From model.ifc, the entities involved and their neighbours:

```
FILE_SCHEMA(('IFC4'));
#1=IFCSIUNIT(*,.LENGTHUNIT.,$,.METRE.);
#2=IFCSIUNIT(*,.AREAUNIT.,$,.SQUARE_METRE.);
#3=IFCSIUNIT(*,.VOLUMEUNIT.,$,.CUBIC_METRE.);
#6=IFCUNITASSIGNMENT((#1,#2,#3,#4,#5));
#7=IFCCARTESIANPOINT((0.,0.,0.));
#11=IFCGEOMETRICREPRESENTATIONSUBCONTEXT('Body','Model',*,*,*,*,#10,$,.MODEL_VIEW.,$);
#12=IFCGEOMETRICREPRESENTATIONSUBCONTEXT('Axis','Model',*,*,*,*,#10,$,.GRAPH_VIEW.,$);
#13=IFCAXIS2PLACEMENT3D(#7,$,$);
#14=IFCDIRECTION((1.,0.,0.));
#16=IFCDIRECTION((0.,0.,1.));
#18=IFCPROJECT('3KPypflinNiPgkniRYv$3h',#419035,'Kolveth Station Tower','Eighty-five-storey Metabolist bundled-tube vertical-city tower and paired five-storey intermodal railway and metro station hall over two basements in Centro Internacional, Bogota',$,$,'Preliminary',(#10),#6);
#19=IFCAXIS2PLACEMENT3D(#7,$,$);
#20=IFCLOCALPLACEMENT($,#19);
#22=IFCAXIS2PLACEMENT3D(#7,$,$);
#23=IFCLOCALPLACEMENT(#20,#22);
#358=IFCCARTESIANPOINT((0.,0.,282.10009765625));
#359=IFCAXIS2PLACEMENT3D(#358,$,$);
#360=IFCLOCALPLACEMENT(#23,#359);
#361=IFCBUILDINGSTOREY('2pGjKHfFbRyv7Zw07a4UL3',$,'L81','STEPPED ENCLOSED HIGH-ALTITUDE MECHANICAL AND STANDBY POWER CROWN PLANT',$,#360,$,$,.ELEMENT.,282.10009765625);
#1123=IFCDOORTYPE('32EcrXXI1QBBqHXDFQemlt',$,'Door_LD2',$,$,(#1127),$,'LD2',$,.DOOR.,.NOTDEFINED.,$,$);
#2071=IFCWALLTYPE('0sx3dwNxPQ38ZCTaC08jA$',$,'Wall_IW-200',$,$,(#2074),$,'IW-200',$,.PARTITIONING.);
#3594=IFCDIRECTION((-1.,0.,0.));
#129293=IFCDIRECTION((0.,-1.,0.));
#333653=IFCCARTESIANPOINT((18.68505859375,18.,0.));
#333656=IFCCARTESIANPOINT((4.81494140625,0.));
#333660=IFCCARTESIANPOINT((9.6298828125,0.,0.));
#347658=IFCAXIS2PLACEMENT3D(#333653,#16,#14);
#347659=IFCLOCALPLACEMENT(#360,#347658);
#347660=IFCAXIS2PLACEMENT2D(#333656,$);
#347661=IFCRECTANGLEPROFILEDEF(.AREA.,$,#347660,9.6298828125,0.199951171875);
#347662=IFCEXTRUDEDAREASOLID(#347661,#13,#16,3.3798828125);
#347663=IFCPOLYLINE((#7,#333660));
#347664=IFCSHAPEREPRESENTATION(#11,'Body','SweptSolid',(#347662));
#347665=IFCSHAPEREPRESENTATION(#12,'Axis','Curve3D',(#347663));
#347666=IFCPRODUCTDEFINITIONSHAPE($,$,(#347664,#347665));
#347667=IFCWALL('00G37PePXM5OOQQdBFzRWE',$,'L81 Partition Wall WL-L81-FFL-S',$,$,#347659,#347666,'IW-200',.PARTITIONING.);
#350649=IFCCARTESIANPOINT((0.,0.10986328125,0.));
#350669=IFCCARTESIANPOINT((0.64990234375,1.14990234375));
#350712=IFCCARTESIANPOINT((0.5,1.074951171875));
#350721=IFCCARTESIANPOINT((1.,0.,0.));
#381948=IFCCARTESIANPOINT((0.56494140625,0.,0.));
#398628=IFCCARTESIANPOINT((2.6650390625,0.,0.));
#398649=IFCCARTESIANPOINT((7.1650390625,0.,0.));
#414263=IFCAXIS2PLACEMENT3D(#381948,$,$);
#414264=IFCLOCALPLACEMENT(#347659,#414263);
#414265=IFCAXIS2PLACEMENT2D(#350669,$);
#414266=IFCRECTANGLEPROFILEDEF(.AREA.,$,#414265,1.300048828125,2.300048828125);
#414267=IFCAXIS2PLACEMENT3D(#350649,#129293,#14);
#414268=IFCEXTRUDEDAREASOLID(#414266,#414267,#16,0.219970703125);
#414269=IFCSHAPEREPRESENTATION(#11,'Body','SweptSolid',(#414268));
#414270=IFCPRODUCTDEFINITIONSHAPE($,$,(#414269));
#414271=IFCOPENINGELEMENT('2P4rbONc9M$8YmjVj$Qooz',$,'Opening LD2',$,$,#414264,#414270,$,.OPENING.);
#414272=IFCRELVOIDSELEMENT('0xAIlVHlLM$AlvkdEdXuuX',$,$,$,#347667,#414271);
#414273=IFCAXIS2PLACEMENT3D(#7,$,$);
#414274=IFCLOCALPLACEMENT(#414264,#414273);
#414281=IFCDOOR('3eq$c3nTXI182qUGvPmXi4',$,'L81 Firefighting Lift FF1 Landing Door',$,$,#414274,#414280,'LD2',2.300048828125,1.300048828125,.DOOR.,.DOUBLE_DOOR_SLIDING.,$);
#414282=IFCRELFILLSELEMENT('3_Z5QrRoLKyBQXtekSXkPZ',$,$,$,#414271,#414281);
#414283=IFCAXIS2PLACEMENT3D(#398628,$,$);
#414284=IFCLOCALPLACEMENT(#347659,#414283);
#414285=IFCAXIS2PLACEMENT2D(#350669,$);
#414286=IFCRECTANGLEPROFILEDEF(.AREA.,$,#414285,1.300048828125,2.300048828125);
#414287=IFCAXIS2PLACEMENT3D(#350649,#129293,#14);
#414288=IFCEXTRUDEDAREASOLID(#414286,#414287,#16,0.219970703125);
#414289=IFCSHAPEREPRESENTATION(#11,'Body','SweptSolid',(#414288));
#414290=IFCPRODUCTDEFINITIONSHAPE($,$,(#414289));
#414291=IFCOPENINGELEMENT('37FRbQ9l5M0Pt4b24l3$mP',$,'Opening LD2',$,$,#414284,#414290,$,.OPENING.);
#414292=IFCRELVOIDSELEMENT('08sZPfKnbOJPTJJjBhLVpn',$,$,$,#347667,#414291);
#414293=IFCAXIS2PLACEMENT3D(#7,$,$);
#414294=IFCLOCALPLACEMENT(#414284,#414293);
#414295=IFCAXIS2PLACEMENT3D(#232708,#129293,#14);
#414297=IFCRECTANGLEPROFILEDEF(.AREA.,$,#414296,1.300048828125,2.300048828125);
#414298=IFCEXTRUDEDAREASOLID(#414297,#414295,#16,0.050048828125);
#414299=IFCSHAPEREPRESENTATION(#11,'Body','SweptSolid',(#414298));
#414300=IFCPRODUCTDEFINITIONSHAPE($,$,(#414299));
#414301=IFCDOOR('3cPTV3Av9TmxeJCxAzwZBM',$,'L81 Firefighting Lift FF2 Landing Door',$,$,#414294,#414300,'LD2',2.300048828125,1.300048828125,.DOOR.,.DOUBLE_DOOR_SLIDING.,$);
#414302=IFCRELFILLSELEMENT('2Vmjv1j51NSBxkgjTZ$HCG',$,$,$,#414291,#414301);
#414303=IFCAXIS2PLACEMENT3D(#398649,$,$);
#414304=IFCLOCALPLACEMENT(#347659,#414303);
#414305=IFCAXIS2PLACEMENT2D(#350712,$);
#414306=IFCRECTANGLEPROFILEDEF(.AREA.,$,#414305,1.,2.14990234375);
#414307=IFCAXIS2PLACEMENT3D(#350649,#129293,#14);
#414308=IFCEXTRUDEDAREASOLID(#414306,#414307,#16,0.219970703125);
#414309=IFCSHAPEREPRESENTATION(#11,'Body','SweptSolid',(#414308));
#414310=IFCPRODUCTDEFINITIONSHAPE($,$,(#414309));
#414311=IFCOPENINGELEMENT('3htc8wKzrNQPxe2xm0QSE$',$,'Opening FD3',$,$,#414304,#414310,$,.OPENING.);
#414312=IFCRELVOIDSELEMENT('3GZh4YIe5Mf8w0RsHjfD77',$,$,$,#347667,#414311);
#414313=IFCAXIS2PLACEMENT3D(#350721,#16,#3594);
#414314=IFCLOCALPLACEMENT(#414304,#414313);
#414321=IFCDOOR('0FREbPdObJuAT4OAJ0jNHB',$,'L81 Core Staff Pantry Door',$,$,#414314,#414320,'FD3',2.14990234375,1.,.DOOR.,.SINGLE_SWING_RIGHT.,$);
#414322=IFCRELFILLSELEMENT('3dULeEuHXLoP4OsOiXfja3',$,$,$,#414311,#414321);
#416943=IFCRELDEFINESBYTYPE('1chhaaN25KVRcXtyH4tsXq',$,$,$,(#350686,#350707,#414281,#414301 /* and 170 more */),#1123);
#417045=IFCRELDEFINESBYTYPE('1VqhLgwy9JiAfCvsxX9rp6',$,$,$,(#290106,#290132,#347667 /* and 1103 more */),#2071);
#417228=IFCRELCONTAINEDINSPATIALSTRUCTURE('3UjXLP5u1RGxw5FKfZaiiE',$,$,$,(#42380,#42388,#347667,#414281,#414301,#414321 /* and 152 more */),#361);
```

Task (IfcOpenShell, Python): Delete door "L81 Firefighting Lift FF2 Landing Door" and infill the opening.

```python
import ifcopenshell
import ifcopenshell.api.feature
import ifcopenshell.api.root
import ifcopenshell.geom
import ifcopenshell.util.shape

model = ifcopenshell.open("model.ifc")
settings = ifcopenshell.geom.settings()


def volume(element):
    """Net volume in cubic metres, openings subtracted."""
    shape = ifcopenshell.geom.create_shape(settings, element)
    return ifcopenshell.util.shape.get_volume(shape.geometry)


door = model.by_guid("3cPTV3Av9TmxeJCxAzwZBM")
opening = door.FillsVoids[0].RelatingOpeningElement
wall = opening.VoidsElements[0].RelatingBuildingElement
before = volume(wall)

ifcopenshell.api.root.remove_product(model, product=door)
ifcopenshell.api.feature.remove_feature(model, feature=opening)

after = volume(wall)

print(f"wall volume {before:.3f} -> {after:.3f} m3")

model.write("model-out.ifc")
```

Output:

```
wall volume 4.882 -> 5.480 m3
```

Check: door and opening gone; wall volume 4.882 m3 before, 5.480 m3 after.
